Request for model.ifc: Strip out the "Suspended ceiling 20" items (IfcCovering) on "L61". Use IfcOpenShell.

First a look at what the model holds.

```python
import ifcopenshell
import ifcopenshell.util.element

model = ifcopenshell.open("model.ifc")
print(model.schema)
storey = next(s for s in model.by_type("IfcBuildingStorey") if s.Name == "L61")
coverings = [e for e in ifcopenshell.util.element.get_decomposition(storey) if e.is_a("IfcCovering")]
seen = {}
for e in coverings:
    element_type = ifcopenshell.util.element.get_type(e)
    name = element_type.Name if element_type not in (None, e) else None
    seen[name] = seen.get(name, 0) + 1
for name, count in sorted(seen.items(), key=str):
    print(count, "x", name)
```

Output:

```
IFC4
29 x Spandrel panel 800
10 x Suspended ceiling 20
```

```python
import ifcopenshell
import ifcopenshell.api.root
import ifcopenshell.util.element

model = ifcopenshell.open("model.ifc")

storey = next(s for s in model.by_type("IfcBuildingStorey") if s.Name == "L61")
coverings = [e for e in ifcopenshell.util.element.get_decomposition(storey) if e.is_a("IfcCovering")]
targets = [e for e in coverings if (t := ifcopenshell.util.element.get_type(e)) not in (None, e) and t.Name == "Suspended ceiling 20"]

for e in targets:
    ifcopenshell.api.root.remove_product(model, product=e)
print(len(targets), "removed")

model.write("model_rev.ifc")
```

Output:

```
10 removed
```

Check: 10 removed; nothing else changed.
